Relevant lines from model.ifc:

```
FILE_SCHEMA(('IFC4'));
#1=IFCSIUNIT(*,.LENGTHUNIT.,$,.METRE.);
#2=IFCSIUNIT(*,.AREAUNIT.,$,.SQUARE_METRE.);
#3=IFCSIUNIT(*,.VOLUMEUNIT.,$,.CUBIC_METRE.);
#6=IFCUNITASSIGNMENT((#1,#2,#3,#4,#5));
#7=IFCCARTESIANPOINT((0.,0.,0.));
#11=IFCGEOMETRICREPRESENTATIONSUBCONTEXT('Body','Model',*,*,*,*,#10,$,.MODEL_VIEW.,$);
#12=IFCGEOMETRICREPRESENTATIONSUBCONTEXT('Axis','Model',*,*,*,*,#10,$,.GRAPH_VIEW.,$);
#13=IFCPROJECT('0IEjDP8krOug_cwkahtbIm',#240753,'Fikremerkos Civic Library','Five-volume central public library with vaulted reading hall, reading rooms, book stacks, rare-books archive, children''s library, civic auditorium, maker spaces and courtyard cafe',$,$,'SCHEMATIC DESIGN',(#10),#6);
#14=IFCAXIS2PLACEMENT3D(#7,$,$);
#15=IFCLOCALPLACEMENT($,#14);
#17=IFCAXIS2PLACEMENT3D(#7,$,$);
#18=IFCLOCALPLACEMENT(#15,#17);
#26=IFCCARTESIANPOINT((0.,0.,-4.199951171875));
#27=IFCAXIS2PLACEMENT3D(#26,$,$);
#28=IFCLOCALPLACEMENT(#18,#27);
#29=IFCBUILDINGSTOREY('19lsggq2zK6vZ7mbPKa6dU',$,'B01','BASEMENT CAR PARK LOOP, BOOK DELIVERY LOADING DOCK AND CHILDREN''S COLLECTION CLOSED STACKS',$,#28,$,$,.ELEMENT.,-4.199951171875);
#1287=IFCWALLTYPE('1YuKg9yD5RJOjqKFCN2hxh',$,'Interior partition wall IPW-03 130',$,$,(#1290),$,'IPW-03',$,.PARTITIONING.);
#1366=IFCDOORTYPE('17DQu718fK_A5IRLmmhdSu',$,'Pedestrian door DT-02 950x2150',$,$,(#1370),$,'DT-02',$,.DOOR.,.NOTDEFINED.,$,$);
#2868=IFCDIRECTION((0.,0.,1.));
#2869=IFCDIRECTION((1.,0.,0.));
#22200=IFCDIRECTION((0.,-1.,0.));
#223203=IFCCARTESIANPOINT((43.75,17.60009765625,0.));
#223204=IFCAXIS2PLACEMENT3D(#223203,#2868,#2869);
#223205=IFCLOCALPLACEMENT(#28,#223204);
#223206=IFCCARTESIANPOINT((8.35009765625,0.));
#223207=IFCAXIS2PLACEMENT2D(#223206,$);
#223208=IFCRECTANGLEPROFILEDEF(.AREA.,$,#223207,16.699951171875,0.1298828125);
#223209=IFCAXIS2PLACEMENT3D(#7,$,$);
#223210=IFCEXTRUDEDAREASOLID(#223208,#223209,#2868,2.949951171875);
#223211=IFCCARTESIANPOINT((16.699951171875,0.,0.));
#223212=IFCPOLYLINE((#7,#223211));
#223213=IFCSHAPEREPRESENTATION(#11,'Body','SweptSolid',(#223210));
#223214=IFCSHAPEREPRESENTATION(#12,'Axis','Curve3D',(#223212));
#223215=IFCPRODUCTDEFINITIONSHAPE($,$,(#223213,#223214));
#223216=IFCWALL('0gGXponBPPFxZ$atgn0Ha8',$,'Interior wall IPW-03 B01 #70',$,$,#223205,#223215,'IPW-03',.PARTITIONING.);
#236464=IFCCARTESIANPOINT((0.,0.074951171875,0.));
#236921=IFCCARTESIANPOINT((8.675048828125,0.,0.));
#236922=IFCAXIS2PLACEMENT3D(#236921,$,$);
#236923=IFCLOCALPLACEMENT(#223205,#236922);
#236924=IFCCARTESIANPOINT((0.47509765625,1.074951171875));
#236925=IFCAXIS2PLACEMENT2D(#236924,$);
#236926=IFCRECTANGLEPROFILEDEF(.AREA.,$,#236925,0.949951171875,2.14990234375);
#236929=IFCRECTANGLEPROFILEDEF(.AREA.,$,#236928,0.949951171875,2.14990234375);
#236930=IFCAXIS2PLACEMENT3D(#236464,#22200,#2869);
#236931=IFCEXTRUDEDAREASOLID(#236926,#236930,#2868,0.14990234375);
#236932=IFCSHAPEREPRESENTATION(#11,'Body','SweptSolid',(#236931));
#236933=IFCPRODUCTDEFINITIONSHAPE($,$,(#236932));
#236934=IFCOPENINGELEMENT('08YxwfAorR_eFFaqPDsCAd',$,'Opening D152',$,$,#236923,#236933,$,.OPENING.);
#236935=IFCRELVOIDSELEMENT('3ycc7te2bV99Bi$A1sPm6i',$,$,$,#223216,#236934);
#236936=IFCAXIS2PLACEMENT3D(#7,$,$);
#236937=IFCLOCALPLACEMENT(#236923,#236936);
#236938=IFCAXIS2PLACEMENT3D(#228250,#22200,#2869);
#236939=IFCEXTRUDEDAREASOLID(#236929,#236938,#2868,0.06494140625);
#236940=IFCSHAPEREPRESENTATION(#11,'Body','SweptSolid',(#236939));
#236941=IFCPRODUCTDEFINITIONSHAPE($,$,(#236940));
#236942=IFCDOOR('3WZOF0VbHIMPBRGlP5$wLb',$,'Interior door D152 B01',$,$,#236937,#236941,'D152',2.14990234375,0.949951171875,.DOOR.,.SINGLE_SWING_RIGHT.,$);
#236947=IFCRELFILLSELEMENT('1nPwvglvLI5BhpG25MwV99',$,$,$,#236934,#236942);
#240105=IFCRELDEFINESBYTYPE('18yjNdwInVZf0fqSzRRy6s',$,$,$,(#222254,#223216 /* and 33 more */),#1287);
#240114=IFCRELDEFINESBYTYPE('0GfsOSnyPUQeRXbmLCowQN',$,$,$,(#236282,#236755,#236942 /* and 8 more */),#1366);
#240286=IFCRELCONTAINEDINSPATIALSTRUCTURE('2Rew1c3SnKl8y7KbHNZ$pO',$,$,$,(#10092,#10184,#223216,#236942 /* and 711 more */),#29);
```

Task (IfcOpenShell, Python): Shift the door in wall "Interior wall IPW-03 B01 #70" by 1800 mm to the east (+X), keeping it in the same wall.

```python
import ifcopenshell
import ifcopenshell.api.geometry
import ifcopenshell.util.placement
import ifcopenshell.util.unit

model = ifcopenshell.open("model.ifc")
unit_scale = ifcopenshell.util.unit.calculate_unit_scale(model)

door = model.by_guid("3WZOF0VbHIMPBRGlP5$wLb")
opening = door.FillsVoids[0].RelatingOpeningElement
wall = opening.VoidsElements[0].RelatingBuildingElement

wall_matrix = ifcopenshell.util.placement.get_local_placement(wall.ObjectPlacement)
shift = wall_matrix[:3, 0] * 1.8 / unit_scale
before = ifcopenshell.util.placement.get_local_placement(door.ObjectPlacement)[:3, 3].copy()

# The door is placed relative to its opening, so it follows when the opening moves.
matrix = ifcopenshell.util.placement.get_local_placement(opening.ObjectPlacement)
matrix[:3, 3] += shift
ifcopenshell.api.geometry.edit_object_placement(
    model, product=opening, matrix=matrix, is_si=False, should_transform_children=True
)

after = ifcopenshell.util.placement.get_local_placement(door.ObjectPlacement)[:3, 3]
print("door moved by", (after - before).round(3) + 0.0)

model.write("model_v2.ifc")
```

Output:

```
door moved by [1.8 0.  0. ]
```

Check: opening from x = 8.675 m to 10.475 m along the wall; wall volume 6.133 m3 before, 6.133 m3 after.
